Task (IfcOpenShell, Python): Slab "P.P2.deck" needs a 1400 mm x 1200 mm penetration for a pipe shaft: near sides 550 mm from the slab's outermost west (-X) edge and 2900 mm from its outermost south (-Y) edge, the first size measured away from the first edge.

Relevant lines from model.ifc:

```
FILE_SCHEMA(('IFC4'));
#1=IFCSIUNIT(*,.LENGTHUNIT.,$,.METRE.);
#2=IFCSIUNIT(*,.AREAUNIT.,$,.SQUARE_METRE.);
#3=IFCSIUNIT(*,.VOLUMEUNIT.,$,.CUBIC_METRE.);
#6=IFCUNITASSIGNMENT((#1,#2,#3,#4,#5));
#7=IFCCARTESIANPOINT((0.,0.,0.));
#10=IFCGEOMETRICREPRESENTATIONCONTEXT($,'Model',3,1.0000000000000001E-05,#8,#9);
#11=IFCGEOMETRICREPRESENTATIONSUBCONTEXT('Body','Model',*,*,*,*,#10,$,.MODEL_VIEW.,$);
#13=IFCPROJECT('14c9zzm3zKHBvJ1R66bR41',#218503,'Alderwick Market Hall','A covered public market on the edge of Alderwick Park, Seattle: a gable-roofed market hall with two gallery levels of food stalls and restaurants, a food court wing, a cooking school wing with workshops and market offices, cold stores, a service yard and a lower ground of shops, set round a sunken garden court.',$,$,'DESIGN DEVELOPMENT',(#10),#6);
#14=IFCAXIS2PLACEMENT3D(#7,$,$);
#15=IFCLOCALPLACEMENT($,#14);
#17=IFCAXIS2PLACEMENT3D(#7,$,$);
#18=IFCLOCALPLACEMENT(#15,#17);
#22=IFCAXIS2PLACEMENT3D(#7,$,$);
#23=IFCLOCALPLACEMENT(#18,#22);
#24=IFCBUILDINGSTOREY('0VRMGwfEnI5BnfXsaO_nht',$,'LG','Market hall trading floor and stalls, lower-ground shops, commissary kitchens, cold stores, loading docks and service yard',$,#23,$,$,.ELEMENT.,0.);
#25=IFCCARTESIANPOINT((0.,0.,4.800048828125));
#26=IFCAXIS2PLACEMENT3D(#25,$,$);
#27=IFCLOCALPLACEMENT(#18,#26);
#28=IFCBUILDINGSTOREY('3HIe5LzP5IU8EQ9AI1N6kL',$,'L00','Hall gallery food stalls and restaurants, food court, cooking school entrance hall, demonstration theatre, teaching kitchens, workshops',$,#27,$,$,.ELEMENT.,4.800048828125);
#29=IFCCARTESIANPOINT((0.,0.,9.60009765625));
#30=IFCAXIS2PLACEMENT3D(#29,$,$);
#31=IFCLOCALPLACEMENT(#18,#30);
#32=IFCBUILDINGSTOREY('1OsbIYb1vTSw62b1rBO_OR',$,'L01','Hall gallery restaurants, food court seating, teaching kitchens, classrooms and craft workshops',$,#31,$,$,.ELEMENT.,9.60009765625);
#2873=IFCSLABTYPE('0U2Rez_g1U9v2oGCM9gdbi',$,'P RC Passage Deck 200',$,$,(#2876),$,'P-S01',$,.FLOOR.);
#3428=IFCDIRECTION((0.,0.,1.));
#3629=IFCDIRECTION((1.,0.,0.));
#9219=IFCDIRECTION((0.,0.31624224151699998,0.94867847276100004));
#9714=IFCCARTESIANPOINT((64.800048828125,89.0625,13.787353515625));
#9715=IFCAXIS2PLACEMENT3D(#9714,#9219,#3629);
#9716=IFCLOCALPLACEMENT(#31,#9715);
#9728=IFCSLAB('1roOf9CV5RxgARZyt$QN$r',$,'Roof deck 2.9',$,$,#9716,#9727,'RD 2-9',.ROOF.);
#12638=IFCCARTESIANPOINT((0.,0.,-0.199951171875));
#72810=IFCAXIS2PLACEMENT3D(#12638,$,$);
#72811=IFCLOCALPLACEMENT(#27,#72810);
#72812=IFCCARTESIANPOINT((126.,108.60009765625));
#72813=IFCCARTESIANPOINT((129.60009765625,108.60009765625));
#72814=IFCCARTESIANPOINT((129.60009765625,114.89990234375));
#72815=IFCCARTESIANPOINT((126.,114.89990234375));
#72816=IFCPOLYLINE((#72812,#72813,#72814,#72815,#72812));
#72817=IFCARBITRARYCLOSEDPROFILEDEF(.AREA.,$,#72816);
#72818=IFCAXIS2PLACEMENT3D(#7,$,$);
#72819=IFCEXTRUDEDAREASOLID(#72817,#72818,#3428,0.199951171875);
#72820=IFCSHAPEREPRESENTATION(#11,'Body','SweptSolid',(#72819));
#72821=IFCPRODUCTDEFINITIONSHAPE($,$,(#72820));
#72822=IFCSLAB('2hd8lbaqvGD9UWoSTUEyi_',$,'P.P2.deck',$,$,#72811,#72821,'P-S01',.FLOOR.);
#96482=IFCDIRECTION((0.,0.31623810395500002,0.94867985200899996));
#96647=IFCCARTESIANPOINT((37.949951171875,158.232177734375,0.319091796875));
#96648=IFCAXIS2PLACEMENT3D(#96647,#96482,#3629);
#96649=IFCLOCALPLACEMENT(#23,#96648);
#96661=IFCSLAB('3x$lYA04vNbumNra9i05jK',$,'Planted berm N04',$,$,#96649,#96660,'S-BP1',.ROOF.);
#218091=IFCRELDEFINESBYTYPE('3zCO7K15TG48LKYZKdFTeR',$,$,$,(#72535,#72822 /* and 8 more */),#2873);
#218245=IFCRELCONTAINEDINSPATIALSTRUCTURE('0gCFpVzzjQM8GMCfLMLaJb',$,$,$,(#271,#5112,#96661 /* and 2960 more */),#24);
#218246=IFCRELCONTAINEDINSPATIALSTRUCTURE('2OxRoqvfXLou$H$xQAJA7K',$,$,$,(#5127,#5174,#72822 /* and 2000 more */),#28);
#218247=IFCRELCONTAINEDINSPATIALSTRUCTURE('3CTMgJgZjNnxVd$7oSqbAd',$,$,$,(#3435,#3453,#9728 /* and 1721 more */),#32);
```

```python
import numpy as np
import ifcopenshell
import ifcopenshell.api.feature
import ifcopenshell.api.geometry
import ifcopenshell.api.root
import ifcopenshell.geom
import ifcopenshell.util.placement
import ifcopenshell.util.representation
import ifcopenshell.util.shape
import ifcopenshell.util.unit

model = ifcopenshell.open("model.ifc")
unit_scale = ifcopenshell.util.unit.calculate_unit_scale(model)
settings = ifcopenshell.geom.settings()


def volume(element):
    """Net volume in cubic metres, openings subtracted."""
    shape = ifcopenshell.geom.create_shape(settings, element)
    return ifcopenshell.util.shape.get_volume(shape.geometry)


slab = model.by_guid("2hd8lbaqvGD9UWoSTUEyi_")
before = volume(slab)

# Extent in the slab's own axes, in metres. The edges named are its -X and -Y sides.
slab_shape = ifcopenshell.geom.create_shape(settings, slab)
vertices = ifcopenshell.util.shape.get_vertices(slab_shape.geometry)
x_min, y_min, bottom = vertices.min(axis=0)
top = vertices[:, 2].max()

opening = ifcopenshell.api.root.create_entity(model, ifc_class="IfcOpeningElement", name="Pipe shaft opening", predefined_type="OPENING")
context = ifcopenshell.util.representation.get_context(model, "Model", "Body", "MODEL_VIEW")
width, depth = 1.4, 1.2
outline = [(0.0, 0.0), (width, 0.0), (width, depth), (0.0, depth), (0.0, 0.0)]
# Overshoot both faces by 50 mm so the cut is clean.
shape = ifcopenshell.api.geometry.add_slab_representation(
    model, context=context, depth=top - bottom + 0.1, polyline=outline
)
ifcopenshell.api.geometry.assign_representation(model, product=opening, representation=shape)

matrix = ifcopenshell.util.placement.get_local_placement(slab.ObjectPlacement)
matrix[:, 3] = matrix @ np.append(np.array([x_min + 0.55, y_min + 2.9, bottom - 0.05]) / unit_scale, 1.0)
ifcopenshell.api.geometry.edit_object_placement(model, product=opening, matrix=matrix, is_si=False)
ifcopenshell.api.feature.add_feature(model, feature=opening, element=slab)

after = volume(slab)

print(f"slab volume {before:.3f} -> {after:.3f} m3")

model.write("model_rev.ifc")
```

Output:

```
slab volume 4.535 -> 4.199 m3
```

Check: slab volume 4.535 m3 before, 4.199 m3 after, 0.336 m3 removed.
